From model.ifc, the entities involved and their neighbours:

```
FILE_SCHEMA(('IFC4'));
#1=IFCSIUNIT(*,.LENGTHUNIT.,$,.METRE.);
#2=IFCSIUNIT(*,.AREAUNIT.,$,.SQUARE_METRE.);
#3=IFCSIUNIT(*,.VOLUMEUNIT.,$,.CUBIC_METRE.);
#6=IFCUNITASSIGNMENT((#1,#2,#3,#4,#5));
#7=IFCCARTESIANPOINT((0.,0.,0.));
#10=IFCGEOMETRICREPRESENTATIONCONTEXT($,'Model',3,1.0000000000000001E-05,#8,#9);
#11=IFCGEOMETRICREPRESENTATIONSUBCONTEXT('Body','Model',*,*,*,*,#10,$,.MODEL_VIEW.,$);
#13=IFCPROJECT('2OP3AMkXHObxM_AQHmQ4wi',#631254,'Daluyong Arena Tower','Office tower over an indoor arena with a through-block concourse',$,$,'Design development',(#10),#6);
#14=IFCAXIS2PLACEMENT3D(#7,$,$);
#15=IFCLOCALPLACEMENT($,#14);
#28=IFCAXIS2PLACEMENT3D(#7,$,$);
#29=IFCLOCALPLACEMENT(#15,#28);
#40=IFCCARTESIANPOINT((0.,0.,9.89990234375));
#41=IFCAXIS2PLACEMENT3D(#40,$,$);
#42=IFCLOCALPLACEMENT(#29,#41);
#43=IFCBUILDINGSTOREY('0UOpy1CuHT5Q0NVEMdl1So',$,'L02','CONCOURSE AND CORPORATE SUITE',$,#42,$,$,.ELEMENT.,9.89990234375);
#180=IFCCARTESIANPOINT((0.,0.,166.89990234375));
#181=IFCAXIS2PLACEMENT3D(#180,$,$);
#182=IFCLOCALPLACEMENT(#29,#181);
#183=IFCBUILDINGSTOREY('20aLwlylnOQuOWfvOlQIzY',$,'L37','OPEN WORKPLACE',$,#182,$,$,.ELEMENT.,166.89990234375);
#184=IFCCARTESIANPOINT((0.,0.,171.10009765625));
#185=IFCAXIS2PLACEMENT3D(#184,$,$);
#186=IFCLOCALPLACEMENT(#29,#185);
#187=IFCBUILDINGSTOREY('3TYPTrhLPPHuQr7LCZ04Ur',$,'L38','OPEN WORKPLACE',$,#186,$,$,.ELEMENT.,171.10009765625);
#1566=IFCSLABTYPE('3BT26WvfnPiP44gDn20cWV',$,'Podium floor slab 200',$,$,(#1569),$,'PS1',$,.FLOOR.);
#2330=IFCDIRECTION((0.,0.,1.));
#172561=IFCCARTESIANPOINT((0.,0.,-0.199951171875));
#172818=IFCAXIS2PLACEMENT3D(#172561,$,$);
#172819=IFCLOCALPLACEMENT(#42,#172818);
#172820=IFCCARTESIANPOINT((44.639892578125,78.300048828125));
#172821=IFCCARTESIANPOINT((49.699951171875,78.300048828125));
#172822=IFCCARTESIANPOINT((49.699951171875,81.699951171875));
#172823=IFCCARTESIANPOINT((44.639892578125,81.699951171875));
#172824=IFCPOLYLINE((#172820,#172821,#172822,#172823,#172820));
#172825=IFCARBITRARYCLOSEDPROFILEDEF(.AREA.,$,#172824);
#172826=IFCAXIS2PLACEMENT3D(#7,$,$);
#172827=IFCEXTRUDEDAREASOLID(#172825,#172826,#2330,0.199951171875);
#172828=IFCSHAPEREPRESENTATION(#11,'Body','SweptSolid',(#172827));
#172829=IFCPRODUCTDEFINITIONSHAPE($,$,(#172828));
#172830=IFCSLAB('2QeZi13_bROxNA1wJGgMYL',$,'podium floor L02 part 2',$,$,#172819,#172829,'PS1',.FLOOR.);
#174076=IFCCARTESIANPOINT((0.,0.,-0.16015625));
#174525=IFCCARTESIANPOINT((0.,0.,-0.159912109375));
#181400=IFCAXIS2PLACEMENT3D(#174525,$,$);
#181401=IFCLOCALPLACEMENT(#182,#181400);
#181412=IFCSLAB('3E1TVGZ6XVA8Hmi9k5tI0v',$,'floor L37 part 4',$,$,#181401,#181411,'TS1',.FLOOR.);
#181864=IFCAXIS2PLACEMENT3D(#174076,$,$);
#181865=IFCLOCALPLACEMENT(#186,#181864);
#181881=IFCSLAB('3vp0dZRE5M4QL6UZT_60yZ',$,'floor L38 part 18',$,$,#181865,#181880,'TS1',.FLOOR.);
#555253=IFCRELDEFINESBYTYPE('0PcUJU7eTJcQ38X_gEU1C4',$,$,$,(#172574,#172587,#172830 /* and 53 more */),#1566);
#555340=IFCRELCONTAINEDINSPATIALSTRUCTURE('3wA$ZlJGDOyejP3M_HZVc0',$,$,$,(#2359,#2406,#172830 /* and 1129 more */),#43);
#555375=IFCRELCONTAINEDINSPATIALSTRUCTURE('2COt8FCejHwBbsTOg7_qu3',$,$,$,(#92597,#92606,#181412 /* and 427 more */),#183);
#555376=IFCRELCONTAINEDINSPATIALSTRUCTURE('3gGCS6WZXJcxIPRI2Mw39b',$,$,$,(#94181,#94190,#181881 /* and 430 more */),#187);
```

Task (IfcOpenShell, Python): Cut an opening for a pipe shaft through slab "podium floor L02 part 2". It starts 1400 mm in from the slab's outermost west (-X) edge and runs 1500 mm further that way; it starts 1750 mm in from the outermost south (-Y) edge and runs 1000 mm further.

```python
import numpy as np
import ifcopenshell
import ifcopenshell.api.feature
import ifcopenshell.api.geometry
import ifcopenshell.api.root
import ifcopenshell.geom
import ifcopenshell.util.placement
import ifcopenshell.util.representation
import ifcopenshell.util.shape
import ifcopenshell.util.unit

model = ifcopenshell.open("model.ifc")
unit_scale = ifcopenshell.util.unit.calculate_unit_scale(model)
settings = ifcopenshell.geom.settings()


def volume(element):
    """Net volume in cubic metres, openings subtracted."""
    shape = ifcopenshell.geom.create_shape(settings, element)
    return ifcopenshell.util.shape.get_volume(shape.geometry)


slab = model.by_guid("2QeZi13_bROxNA1wJGgMYL")
before = volume(slab)

# Extent in the slab's own axes, in metres. The edges named are its -X and -Y sides.
slab_shape = ifcopenshell.geom.create_shape(settings, slab)
vertices = ifcopenshell.util.shape.get_vertices(slab_shape.geometry)
x_min, y_min, bottom = vertices.min(axis=0)
top = vertices[:, 2].max()

opening = ifcopenshell.api.root.create_entity(model, ifc_class="IfcOpeningElement", name="Pipe shaft opening", predefined_type="OPENING")
context = ifcopenshell.util.representation.get_context(model, "Model", "Body", "MODEL_VIEW")
width, depth = 1.5, 1
outline = [(0.0, 0.0), (width, 0.0), (width, depth), (0.0, depth), (0.0, 0.0)]
# Overshoot both faces by 50 mm so the cut is clean.
shape = ifcopenshell.api.geometry.add_slab_representation(
    model, context=context, depth=top - bottom + 0.1, polyline=outline
)
ifcopenshell.api.geometry.assign_representation(model, product=opening, representation=shape)

matrix = ifcopenshell.util.placement.get_local_placement(slab.ObjectPlacement)
matrix[:, 3] = matrix @ np.append(np.array([x_min + 1.4, y_min + 1.75, bottom - 0.05]) / unit_scale, 1.0)
ifcopenshell.api.geometry.edit_object_placement(model, product=opening, matrix=matrix, is_si=False)
ifcopenshell.api.feature.add_feature(model, feature=opening, element=slab)

after = volume(slab)

print(f"slab volume {before:.3f} -> {after:.3f} m3")

model.write("model_updated.ifc")
```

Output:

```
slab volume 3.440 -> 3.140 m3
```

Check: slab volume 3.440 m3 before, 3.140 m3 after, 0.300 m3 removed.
